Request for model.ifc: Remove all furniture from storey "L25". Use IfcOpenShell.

First a look at what the model holds.

```python
import ifcopenshell
import ifcopenshell.util.element

model = ifcopenshell.open("model.ifc")
print(model.schema)
storey = next(s for s in model.by_type("IfcBuildingStorey") if s.Name == "L25")
furniture = [e for e in ifcopenshell.util.element.get_decomposition(storey) if e.is_a("IfcFurnishingElement")]
seen = {}
for e in furniture:
    element_type = ifcopenshell.util.element.get_type(e)
    name = element_type.Name if element_type not in (None, e) else None
    seen[name] = seen.get(name, 0) + 1
for name, count in sorted(seen.items(), key=str):
    print(count, "x", name)
```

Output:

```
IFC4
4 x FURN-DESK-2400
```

```python
import ifcopenshell
import ifcopenshell.api.root
import ifcopenshell.util.element

model = ifcopenshell.open("model.ifc")

storey = next(s for s in model.by_type("IfcBuildingStorey") if s.Name == "L25")
furniture = [e for e in ifcopenshell.util.element.get_decomposition(storey) if e.is_a("IfcFurnishingElement")]

for e in furniture:
    ifcopenshell.api.root.remove_product(model, product=e)
print(len(furniture), "removed")

model.write("model_updated.ifc")
```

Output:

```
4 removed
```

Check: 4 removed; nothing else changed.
